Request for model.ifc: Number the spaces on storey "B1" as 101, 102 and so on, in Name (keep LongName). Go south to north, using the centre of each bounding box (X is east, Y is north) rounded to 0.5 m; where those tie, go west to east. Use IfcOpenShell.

First a look at what the model holds.

```python
import ifcopenshell
import ifcopenshell.util.element
import ifcopenshell.util.placement

model = ifcopenshell.open("model.ifc")
print(model.schema)
storey = next(s for s in model.by_type("IfcBuildingStorey") if s.Name == "B1")
spaces = [e for e in ifcopenshell.util.element.get_decomposition(storey) if e.is_a("IfcSpace")]
for e in sorted(spaces, key=lambda e: e.id()):
    origin = ifcopenshell.util.placement.get_local_placement(e.ObjectPlacement)[:3, 3]
    print(e.id(), e.Name, e.LongName, origin.round(2) + 0.0, sep=" | ")
```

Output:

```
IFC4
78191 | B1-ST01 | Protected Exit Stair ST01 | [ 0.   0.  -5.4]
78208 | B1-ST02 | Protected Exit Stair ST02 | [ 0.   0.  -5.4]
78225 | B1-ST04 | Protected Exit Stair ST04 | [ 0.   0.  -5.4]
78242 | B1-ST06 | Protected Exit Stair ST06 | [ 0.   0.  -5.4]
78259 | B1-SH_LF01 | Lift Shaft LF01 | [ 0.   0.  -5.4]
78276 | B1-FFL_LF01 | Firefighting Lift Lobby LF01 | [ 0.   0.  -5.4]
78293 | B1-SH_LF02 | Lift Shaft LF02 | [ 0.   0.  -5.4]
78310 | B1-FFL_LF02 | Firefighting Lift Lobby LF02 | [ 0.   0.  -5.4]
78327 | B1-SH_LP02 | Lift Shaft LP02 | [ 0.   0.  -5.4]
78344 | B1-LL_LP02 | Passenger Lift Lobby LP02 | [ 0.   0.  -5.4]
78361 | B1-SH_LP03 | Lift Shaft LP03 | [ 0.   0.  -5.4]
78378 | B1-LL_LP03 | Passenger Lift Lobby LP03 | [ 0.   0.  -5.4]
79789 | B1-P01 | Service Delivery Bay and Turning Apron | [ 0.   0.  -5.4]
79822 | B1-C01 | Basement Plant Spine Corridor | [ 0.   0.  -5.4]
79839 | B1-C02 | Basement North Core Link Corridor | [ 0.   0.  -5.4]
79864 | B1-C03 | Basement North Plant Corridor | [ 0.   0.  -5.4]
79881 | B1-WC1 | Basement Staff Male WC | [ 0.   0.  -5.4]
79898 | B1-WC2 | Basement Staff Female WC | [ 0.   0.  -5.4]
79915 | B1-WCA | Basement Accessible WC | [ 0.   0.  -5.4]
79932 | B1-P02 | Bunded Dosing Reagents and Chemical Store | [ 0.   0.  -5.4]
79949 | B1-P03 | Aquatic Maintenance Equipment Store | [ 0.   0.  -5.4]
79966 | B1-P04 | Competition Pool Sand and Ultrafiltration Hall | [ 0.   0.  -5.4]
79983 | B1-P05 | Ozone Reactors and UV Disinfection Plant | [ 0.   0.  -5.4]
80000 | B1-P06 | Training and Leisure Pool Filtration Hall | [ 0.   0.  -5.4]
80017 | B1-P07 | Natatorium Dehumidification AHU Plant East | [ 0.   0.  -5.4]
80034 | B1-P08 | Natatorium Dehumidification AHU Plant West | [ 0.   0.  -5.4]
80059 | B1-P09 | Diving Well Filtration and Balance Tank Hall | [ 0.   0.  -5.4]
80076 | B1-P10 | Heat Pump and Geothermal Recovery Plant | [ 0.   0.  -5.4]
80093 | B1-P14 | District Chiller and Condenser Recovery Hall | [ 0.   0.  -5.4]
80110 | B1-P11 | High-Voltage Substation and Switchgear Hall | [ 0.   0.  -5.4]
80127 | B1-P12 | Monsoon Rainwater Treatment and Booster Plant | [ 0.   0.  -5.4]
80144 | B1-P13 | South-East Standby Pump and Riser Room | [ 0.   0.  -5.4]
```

```python
import ifcopenshell
import ifcopenshell.geom
import ifcopenshell.util.element
import ifcopenshell.util.shape

model = ifcopenshell.open("model.ifc")
settings = ifcopenshell.geom.settings()
settings.set("use-world-coords", True)


def centre(element):
    shape = ifcopenshell.geom.create_shape(settings, element)
    return ifcopenshell.util.shape.get_bbox_centroid(shape.geometry)


storey = next(s for s in model.by_type("IfcBuildingStorey") if s.Name == "B1")
spaces = [e for e in ifcopenshell.util.element.get_decomposition(storey) if e.is_a("IfcSpace")]

# Insertion points can sit at a corner or the storey origin, so sort by the geometry (in metres).
centres = {e: centre(e) for e in spaces}
spaces.sort(key=lambda e: (round(centres[e][1] / 0.5), centres[e][0]))

for i, e in enumerate(spaces, start=1):
    number = f"1{i:02d}"
    e.Name = number
    print(e.id(), number)

model.write("model_rev.ifc")
```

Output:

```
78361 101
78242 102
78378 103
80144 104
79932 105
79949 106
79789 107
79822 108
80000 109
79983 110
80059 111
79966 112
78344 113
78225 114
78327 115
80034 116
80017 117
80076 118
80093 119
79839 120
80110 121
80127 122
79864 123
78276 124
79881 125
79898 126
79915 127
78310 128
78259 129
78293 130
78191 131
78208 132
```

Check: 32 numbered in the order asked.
